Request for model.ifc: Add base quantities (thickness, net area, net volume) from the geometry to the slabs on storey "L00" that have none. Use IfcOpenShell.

First a look at what the model holds.

```python
import ifcopenshell
import ifcopenshell.util.element
import ifcopenshell.util.unit

model = ifcopenshell.open("model.ifc")
print(model.schema)
for unit_type in ("LENGTHUNIT", "AREAUNIT", "VOLUMEUNIT"):
    print(unit_type, ifcopenshell.util.unit.calculate_unit_scale(model, unit_type))
storey = next(s for s in model.by_type("IfcBuildingStorey") if s.Name == "L00")
slabs = [e for e in ifcopenshell.util.element.get_decomposition(storey) if e.is_a("IfcSlab")]
for e in sorted(slabs, key=lambda e: e.id()):
    print(e.id(), e.is_a(), e.Name, list(ifcopenshell.util.element.get_psets(e, qtos_only=True)), sep=" | ")
```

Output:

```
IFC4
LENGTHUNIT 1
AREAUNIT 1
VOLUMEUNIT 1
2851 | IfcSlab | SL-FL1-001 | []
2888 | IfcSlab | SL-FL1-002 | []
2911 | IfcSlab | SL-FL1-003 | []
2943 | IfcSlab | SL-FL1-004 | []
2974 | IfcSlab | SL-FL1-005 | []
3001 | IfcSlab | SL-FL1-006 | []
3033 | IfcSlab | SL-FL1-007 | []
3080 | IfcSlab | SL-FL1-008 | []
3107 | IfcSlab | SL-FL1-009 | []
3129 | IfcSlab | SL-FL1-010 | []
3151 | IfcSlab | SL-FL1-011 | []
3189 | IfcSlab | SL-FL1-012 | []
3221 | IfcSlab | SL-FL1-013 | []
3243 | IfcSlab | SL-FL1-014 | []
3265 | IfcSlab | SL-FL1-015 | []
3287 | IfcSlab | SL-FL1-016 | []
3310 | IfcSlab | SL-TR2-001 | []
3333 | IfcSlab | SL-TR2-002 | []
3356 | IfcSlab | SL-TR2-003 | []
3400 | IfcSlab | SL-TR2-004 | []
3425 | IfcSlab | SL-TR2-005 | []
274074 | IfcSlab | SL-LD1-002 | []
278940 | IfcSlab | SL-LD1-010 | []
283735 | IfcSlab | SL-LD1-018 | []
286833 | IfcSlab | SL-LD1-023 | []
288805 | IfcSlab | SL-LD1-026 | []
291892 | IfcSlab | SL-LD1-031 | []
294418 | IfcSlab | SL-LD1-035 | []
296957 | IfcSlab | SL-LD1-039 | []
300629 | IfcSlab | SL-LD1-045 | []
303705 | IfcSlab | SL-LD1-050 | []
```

```python
import ifcopenshell
import ifcopenshell.api.pset
import ifcopenshell.geom
import ifcopenshell.util.element
import ifcopenshell.util.shape
import ifcopenshell.util.unit

model = ifcopenshell.open("model.ifc")
unit_scale = ifcopenshell.util.unit.calculate_unit_scale(model)
area_scale = ifcopenshell.util.unit.calculate_unit_scale(model, "AREAUNIT")
volume_scale = ifcopenshell.util.unit.calculate_unit_scale(model, "VOLUMEUNIT")
settings = ifcopenshell.geom.settings()

storey = next(s for s in model.by_type("IfcBuildingStorey") if s.Name == "L00")
slabs = [e for e in ifcopenshell.util.element.get_decomposition(storey) if e.is_a("IfcSlab")]

for e in sorted(slabs, key=lambda e: e.id()):
    if ifcopenshell.util.element.get_psets(e, qtos_only=True, should_inherit=False):
        continue
    # Geometry comes back in metres, in the element's own axes.
    shape = ifcopenshell.geom.create_shape(settings, e)
    values = {
        "Width": ifcopenshell.util.shape.get_z(shape.geometry) / unit_scale,
        "NetArea": ifcopenshell.util.shape.get_footprint_area(shape.geometry) / area_scale,
        "NetVolume": ifcopenshell.util.shape.get_volume(shape.geometry) / volume_scale,
    }
    qto = ifcopenshell.api.pset.add_qto(model, product=e, name="Qto_SlabBaseQuantities")
    ifcopenshell.api.pset.edit_qto(model, qto=qto, properties=values)
    print(e.id(), {k: round(v, 3) for k, v in values.items()})

model.write("model_edited.ifc")
```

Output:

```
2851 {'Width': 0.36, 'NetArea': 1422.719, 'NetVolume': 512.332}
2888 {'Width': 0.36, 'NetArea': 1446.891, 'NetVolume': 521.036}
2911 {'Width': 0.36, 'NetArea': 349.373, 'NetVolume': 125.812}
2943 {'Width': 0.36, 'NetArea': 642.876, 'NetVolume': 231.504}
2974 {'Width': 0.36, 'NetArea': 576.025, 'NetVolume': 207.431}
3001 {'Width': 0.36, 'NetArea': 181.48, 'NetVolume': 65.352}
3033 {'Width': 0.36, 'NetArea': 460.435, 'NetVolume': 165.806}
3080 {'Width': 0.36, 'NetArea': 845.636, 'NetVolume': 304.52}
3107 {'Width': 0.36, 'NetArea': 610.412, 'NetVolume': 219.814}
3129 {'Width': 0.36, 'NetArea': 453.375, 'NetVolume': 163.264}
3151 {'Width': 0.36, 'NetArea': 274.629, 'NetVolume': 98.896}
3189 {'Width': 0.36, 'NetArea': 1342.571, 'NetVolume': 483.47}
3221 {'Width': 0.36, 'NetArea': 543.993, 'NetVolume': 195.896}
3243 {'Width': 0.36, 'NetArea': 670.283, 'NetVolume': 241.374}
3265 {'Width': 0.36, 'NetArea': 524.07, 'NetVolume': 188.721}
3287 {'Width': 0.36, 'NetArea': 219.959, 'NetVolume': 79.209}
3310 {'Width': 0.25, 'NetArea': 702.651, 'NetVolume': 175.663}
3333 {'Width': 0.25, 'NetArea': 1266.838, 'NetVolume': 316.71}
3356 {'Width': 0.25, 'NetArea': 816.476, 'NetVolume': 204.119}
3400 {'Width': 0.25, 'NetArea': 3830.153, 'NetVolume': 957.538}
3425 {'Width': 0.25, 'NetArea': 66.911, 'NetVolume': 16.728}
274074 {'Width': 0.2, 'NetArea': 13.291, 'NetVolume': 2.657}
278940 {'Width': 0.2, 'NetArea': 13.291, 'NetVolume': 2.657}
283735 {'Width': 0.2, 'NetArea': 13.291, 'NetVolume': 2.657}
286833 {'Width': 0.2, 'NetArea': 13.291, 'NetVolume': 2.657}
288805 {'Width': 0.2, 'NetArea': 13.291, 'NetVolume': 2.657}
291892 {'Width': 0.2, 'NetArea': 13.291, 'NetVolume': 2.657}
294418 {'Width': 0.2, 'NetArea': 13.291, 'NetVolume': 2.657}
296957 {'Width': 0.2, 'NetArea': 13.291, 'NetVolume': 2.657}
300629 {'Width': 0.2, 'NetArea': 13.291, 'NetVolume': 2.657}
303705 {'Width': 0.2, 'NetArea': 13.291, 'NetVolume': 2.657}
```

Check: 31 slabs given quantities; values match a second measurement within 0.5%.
